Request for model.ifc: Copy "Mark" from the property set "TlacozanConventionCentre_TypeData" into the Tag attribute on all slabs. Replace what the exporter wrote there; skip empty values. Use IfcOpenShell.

First a look at what the model holds.

```python
import ifcopenshell
import ifcopenshell.util.element

model = ifcopenshell.open("model.ifc")
print(model.schema)
slabs = model.by_type("IfcSlab")
print(len(slabs), "slabs")
for e in slabs[:8]:
    source = ifcopenshell.util.element.get_pset(e, "TlacozanConventionCentre_TypeData", "Mark")
    target = e.Tag
    print(e.id(), repr(source), repr(target), sep=" | ")
```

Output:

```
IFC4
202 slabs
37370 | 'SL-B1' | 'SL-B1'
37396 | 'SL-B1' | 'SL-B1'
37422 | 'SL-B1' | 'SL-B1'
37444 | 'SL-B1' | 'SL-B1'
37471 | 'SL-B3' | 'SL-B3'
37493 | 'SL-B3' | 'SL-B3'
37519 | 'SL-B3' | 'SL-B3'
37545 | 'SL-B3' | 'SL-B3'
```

```python
import ifcopenshell
import ifcopenshell.util.element

model = ifcopenshell.open("model.ifc")

count = 0
for e in model.by_type("IfcSlab"):
    value = ifcopenshell.util.element.get_pset(e, "TlacozanConventionCentre_TypeData", "Mark")
    current = e.Tag
    if not value or not value.strip() or current == value:
        continue
    e.Tag = value
    count += 1

print(count, "slabs updated")

model.write("model_v2.ifc")
```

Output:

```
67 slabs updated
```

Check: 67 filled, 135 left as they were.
